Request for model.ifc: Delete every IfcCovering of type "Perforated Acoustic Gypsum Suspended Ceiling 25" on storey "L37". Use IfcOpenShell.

First a look at what the model holds.

```python
import ifcopenshell
import ifcopenshell.util.element

model = ifcopenshell.open("model.ifc")
print(model.schema)
storey = next(s for s in model.by_type("IfcBuildingStorey") if s.Name == "L37")
coverings = [e for e in ifcopenshell.util.element.get_decomposition(storey) if e.is_a("IfcCovering")]
seen = {}
for e in coverings:
    element_type = ifcopenshell.util.element.get_type(e)
    name = element_type.Name if element_type not in (None, e) else None
    seen[name] = seen.get(name, 0) + 1
for name, count in sorted(seen.items(), key=str):
    print(count, "x", name)
```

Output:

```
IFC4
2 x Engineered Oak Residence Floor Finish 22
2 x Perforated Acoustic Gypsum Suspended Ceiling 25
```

```python
import ifcopenshell
import ifcopenshell.api.root
import ifcopenshell.util.element

model = ifcopenshell.open("model.ifc")

storey = next(s for s in model.by_type("IfcBuildingStorey") if s.Name == "L37")
coverings = [e for e in ifcopenshell.util.element.get_decomposition(storey) if e.is_a("IfcCovering")]
targets = [e for e in coverings if (t := ifcopenshell.util.element.get_type(e)) not in (None, e) and t.Name == "Perforated Acoustic Gypsum Suspended Ceiling 25"]

for e in targets:
    ifcopenshell.api.root.remove_product(model, product=e)
print(len(targets), "removed")

model.write("model_updated.ifc")
```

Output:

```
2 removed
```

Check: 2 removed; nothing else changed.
